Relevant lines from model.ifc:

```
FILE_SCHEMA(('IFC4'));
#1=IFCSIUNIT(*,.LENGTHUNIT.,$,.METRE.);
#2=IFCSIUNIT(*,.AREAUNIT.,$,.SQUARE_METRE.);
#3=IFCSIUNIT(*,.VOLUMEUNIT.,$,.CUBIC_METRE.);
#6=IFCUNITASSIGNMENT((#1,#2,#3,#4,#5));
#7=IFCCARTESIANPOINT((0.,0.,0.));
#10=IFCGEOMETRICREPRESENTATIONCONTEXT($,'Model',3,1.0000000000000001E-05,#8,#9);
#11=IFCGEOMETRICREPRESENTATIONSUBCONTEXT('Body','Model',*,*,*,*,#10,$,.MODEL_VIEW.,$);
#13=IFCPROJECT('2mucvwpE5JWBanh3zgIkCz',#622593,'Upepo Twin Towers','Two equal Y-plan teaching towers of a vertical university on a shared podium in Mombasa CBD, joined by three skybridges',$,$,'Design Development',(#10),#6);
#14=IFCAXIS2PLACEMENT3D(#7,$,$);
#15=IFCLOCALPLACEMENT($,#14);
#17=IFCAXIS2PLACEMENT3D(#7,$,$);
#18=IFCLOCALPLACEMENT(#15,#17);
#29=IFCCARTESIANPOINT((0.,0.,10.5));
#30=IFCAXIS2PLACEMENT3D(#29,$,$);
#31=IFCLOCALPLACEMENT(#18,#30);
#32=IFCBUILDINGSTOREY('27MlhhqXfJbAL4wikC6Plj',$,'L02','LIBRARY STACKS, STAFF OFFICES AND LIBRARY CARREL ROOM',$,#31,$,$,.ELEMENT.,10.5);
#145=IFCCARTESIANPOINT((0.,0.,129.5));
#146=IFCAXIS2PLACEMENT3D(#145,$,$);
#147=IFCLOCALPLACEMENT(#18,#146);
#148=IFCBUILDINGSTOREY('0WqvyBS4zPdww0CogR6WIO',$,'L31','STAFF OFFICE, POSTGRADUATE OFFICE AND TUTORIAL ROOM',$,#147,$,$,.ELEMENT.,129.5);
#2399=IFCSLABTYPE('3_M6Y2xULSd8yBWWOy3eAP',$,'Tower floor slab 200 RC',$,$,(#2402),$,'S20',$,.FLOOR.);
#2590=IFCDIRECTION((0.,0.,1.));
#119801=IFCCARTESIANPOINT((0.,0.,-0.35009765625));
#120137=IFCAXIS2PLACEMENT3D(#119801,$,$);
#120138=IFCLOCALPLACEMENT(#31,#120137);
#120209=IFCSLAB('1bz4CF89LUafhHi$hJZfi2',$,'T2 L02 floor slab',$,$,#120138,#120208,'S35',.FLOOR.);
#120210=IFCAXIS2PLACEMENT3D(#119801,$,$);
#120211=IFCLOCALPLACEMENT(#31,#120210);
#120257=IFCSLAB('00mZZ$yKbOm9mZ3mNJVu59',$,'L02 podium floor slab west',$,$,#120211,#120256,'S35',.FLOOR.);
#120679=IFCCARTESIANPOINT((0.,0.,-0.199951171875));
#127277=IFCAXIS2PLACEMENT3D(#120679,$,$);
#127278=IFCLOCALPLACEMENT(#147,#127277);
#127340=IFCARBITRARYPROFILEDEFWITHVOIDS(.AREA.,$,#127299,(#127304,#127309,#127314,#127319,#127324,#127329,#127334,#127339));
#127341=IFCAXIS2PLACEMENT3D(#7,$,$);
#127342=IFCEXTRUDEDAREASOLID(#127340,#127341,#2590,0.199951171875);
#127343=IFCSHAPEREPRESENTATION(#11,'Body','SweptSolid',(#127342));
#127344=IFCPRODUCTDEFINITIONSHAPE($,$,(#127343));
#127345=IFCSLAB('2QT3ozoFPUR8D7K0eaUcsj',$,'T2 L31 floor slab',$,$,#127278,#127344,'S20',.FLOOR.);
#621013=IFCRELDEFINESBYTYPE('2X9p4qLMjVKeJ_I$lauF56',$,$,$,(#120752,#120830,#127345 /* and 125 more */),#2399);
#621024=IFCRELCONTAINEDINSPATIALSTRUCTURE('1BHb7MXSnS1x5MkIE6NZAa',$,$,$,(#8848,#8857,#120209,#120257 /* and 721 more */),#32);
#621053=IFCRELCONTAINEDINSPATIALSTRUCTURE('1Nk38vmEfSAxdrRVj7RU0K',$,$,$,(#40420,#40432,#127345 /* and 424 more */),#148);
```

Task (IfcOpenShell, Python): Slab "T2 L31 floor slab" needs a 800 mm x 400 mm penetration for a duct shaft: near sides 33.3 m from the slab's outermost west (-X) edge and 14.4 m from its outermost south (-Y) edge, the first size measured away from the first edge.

```python
import numpy as np
import ifcopenshell
import ifcopenshell.api.feature
import ifcopenshell.api.geometry
import ifcopenshell.api.root
import ifcopenshell.geom
import ifcopenshell.util.placement
import ifcopenshell.util.representation
import ifcopenshell.util.shape
import ifcopenshell.util.unit

model = ifcopenshell.open("model.ifc")
unit_scale = ifcopenshell.util.unit.calculate_unit_scale(model)
settings = ifcopenshell.geom.settings()


def volume(element):
    """Net volume in cubic metres, openings subtracted."""
    shape = ifcopenshell.geom.create_shape(settings, element)
    return ifcopenshell.util.shape.get_volume(shape.geometry)


slab = model.by_guid("2QT3ozoFPUR8D7K0eaUcsj")
before = volume(slab)

# Extent in the slab's own axes, in metres. The edges named are its -X and -Y sides.
slab_shape = ifcopenshell.geom.create_shape(settings, slab)
vertices = ifcopenshell.util.shape.get_vertices(slab_shape.geometry)
x_min, y_min, bottom = vertices.min(axis=0)
top = vertices[:, 2].max()

opening = ifcopenshell.api.root.create_entity(model, ifc_class="IfcOpeningElement", name="Duct shaft opening", predefined_type="OPENING")
context = ifcopenshell.util.representation.get_context(model, "Model", "Body", "MODEL_VIEW")
width, depth = 0.8, 0.4
outline = [(0.0, 0.0), (width, 0.0), (width, depth), (0.0, depth), (0.0, 0.0)]
# Overshoot both faces by 50 mm so the cut is clean.
shape = ifcopenshell.api.geometry.add_slab_representation(
    model, context=context, depth=top - bottom + 0.1, polyline=outline
)
ifcopenshell.api.geometry.assign_representation(model, product=opening, representation=shape)

matrix = ifcopenshell.util.placement.get_local_placement(slab.ObjectPlacement)
matrix[:, 3] = matrix @ np.append(np.array([x_min + 33.3, y_min + 14.4, bottom - 0.05]) / unit_scale, 1.0)
ifcopenshell.api.geometry.edit_object_placement(model, product=opening, matrix=matrix, is_si=False)
ifcopenshell.api.feature.add_feature(model, feature=opening, element=slab)

after = volume(slab)

print(f"slab volume {before:.3f} -> {after:.3f} m3")

model.write("model-out.ifc")
```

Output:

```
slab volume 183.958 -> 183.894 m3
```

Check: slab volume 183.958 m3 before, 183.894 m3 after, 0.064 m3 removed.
